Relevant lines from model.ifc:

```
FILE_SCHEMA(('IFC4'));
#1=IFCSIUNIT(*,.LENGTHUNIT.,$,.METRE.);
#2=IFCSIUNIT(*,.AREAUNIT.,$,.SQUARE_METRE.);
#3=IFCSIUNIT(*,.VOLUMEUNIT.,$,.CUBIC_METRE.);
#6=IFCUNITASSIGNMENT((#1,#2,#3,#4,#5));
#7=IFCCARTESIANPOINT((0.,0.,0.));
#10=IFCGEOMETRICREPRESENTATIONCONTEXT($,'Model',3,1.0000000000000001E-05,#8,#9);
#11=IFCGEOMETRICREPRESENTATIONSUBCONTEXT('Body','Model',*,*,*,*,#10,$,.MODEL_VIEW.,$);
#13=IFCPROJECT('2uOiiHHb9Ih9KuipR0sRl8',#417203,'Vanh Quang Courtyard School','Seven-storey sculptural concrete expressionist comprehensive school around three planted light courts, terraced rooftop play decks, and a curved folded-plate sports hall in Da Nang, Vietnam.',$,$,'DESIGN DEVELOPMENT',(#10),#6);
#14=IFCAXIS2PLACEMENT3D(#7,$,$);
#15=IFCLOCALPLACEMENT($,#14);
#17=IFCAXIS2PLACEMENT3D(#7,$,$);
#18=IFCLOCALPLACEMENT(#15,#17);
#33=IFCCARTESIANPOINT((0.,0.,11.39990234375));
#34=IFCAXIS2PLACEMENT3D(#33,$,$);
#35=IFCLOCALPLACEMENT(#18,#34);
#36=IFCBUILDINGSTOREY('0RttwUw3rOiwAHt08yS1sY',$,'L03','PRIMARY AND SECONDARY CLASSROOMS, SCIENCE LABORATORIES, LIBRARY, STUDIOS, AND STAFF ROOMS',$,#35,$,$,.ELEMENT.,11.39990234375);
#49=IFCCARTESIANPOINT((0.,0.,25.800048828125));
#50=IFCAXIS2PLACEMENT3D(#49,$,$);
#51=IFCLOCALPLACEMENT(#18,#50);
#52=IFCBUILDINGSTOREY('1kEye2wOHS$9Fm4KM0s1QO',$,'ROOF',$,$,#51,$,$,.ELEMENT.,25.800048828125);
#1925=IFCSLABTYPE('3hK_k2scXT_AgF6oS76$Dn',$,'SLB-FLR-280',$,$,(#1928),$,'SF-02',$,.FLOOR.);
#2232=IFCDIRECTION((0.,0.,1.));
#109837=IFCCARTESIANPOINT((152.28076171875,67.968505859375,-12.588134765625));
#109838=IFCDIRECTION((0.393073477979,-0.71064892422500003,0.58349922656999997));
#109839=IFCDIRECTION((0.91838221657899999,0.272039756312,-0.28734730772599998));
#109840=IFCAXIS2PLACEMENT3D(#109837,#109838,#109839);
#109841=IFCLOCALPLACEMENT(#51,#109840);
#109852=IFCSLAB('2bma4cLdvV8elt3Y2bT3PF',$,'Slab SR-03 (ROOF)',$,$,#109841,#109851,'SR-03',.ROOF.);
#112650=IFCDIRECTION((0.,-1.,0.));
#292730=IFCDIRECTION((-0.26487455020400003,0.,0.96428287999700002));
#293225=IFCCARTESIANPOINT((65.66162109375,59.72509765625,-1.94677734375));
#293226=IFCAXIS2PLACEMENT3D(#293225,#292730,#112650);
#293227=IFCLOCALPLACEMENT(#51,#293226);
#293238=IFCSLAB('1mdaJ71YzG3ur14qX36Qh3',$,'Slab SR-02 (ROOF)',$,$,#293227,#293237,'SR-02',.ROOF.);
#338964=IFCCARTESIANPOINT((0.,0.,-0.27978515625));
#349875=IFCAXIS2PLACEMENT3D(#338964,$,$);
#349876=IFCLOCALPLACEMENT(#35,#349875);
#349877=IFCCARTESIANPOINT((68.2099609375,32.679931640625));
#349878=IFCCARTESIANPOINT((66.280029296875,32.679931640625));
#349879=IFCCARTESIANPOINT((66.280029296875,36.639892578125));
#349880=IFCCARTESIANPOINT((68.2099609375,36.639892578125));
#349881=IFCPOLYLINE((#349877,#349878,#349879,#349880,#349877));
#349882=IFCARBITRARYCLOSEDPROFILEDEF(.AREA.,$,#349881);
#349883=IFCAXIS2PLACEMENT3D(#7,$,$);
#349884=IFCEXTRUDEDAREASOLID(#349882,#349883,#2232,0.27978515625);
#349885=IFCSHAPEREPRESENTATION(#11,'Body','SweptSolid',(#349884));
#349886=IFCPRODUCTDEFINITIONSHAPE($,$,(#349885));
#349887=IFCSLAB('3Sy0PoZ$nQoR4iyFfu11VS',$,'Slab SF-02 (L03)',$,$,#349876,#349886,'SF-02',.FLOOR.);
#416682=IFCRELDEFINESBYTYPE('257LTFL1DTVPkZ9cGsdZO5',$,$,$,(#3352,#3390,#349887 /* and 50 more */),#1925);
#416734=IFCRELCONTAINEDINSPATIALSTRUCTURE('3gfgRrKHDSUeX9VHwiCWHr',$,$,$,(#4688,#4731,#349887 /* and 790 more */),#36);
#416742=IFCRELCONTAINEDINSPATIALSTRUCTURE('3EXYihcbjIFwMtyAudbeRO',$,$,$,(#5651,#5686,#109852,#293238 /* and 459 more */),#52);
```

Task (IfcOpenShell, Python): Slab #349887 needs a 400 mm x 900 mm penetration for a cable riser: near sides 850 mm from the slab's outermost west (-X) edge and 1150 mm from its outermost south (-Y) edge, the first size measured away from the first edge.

```python
import numpy as np
import ifcopenshell
import ifcopenshell.api.feature
import ifcopenshell.api.geometry
import ifcopenshell.api.root
import ifcopenshell.geom
import ifcopenshell.util.placement
import ifcopenshell.util.representation
import ifcopenshell.util.shape
import ifcopenshell.util.unit

model = ifcopenshell.open("model.ifc")
unit_scale = ifcopenshell.util.unit.calculate_unit_scale(model)
settings = ifcopenshell.geom.settings()


def volume(element):
    """Net volume in cubic metres, openings subtracted."""
    shape = ifcopenshell.geom.create_shape(settings, element)
    return ifcopenshell.util.shape.get_volume(shape.geometry)


slab = model.by_guid("3Sy0PoZ$nQoR4iyFfu11VS")
before = volume(slab)

# Extent in the slab's own axes, in metres. The edges named are its -X and -Y sides.
slab_shape = ifcopenshell.geom.create_shape(settings, slab)
vertices = ifcopenshell.util.shape.get_vertices(slab_shape.geometry)
x_min, y_min, bottom = vertices.min(axis=0)
top = vertices[:, 2].max()

opening = ifcopenshell.api.root.create_entity(model, ifc_class="IfcOpeningElement", name="Cable riser opening", predefined_type="OPENING")
context = ifcopenshell.util.representation.get_context(model, "Model", "Body", "MODEL_VIEW")
width, depth = 0.4, 0.9
outline = [(0.0, 0.0), (width, 0.0), (width, depth), (0.0, depth), (0.0, 0.0)]
# Overshoot both faces by 50 mm so the cut is clean.
shape = ifcopenshell.api.geometry.add_slab_representation(
    model, context=context, depth=top - bottom + 0.1, polyline=outline
)
ifcopenshell.api.geometry.assign_representation(model, product=opening, representation=shape)

matrix = ifcopenshell.util.placement.get_local_placement(slab.ObjectPlacement)
matrix[:, 3] = matrix @ np.append(np.array([x_min + 0.85, y_min + 1.15, bottom - 0.05]) / unit_scale, 1.0)
ifcopenshell.api.geometry.edit_object_placement(model, product=opening, matrix=matrix, is_si=False)
ifcopenshell.api.feature.add_feature(model, feature=opening, element=slab)

after = volume(slab)

print(f"slab volume {before:.3f} -> {after:.3f} m3")

model.write("model_edited.ifc")
```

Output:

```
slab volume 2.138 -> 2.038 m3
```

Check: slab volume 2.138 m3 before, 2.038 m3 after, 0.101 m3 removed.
